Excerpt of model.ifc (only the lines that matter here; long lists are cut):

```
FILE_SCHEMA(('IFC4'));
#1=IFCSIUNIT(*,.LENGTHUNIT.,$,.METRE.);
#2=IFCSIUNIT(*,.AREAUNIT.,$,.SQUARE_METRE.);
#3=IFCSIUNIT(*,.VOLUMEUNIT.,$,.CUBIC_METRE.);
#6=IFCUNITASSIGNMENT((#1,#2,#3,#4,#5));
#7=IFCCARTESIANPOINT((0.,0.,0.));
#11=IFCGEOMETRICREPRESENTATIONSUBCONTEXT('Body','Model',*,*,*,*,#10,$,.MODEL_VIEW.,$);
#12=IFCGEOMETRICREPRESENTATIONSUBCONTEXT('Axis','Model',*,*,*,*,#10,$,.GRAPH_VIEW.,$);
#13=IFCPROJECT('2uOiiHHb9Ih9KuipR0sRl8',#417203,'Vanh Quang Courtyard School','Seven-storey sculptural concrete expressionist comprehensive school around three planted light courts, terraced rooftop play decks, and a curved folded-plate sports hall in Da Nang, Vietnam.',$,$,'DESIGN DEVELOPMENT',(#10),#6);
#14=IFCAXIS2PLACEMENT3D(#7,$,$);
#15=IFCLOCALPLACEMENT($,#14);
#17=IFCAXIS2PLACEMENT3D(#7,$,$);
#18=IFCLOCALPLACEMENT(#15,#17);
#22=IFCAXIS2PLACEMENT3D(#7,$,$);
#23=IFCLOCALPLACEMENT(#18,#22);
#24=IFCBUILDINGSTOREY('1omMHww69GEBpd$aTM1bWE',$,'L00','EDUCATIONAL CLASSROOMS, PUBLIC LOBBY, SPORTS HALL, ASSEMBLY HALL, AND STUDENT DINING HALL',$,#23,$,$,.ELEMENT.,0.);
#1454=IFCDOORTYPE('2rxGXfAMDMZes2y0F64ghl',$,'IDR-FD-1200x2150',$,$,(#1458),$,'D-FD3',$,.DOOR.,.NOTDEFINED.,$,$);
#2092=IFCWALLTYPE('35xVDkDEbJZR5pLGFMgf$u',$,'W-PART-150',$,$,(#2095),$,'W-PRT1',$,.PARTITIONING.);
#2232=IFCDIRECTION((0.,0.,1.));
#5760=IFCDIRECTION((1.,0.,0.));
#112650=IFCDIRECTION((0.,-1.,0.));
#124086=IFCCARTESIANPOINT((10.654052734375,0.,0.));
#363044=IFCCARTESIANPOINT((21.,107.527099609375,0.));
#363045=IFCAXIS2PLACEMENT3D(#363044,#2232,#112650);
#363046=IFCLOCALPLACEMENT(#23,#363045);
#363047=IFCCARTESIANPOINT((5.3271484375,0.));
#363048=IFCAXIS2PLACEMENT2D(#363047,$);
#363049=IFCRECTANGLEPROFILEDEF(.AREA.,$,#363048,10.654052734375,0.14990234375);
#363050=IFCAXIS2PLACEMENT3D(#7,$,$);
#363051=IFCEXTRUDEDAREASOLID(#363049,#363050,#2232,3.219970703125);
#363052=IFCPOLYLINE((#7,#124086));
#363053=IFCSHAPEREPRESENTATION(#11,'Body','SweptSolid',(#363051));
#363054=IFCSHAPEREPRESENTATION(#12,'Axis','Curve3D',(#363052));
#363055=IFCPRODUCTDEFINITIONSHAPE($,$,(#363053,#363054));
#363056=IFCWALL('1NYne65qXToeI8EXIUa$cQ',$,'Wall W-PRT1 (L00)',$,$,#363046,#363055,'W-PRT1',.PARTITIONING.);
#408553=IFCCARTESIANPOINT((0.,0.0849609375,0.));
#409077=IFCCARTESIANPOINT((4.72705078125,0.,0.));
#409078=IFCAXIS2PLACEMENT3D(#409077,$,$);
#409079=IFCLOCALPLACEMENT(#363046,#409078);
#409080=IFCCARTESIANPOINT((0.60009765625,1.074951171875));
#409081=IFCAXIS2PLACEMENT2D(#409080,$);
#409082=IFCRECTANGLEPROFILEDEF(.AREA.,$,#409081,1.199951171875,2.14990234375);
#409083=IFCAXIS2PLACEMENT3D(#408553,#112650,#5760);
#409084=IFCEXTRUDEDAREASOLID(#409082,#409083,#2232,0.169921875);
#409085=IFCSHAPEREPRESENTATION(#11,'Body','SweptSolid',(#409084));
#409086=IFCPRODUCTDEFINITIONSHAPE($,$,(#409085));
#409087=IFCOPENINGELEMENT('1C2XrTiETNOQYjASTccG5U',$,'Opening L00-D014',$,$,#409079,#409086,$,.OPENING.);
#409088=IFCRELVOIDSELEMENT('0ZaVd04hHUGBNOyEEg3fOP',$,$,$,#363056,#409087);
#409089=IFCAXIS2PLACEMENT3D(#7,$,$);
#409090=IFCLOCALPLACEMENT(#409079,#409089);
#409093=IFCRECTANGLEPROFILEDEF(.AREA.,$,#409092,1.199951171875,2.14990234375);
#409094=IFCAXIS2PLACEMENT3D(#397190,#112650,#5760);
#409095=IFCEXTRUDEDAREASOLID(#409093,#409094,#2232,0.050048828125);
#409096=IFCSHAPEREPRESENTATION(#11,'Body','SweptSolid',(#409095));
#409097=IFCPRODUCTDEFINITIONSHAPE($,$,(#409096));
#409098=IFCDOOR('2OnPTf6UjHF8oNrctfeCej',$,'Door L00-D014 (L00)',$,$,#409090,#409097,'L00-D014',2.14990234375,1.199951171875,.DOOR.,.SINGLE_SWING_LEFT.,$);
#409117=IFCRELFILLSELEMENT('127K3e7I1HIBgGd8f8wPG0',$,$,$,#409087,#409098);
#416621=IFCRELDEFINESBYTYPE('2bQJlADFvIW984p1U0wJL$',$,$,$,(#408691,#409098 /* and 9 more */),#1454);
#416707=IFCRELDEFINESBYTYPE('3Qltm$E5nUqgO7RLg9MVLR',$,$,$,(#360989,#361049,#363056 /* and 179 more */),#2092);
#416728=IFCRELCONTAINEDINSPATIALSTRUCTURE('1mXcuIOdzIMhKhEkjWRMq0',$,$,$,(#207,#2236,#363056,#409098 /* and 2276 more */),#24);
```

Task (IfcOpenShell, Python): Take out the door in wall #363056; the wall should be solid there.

```python
import ifcopenshell
import ifcopenshell.api.feature
import ifcopenshell.api.root
import ifcopenshell.geom
import ifcopenshell.util.shape

model = ifcopenshell.open("model.ifc")
settings = ifcopenshell.geom.settings()


def volume(element):
    """Net volume in cubic metres, openings subtracted."""
    shape = ifcopenshell.geom.create_shape(settings, element)
    return ifcopenshell.util.shape.get_volume(shape.geometry)


door = model.by_id(409098)
opening = door.FillsVoids[0].RelatingOpeningElement
wall = opening.VoidsElements[0].RelatingBuildingElement
before = volume(wall)

ifcopenshell.api.root.remove_product(model, product=door)
ifcopenshell.api.feature.remove_feature(model, feature=opening)

after = volume(wall)

print(f"wall volume {before:.3f} -> {after:.3f} m3")

model.write("model_edited.ifc")
```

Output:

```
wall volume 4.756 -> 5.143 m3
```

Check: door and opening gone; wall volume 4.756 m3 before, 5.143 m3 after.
